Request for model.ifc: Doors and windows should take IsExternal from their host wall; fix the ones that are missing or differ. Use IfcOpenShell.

First a look at what the model holds.

```python
import ifcopenshell
import ifcopenshell.util.element

model = ifcopenshell.open("model.ifc")
print(model.schema)
seen = {}
for e in model.by_type("IfcDoor") + model.by_type("IfcWindow"):
    if not e.FillsVoids:
        continue
    host = e.FillsVoids[0].RelatingOpeningElement.VoidsElements[0].RelatingBuildingElement
    own = ifcopenshell.util.element.get_pset(e, f"Pset_{e.is_a()[3:].removesuffix('StandardCase')}Common", "IsExternal")
    wall = ifcopenshell.util.element.get_pset(host, "Pset_WallCommon", "IsExternal")
    seen[e.is_a(), own, wall] = seen.get((e.is_a(), own, wall), 0) + 1
for (cls, own, wall), count in sorted(seen.items(), key=str):
    print(count, cls, "IsExternal:", own, "| host wall:", wall)
```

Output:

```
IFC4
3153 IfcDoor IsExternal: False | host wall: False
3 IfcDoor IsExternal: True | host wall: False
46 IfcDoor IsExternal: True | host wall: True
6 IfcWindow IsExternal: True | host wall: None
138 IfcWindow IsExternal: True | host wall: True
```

```python
import ifcopenshell
import ifcopenshell.api.pset
import ifcopenshell.util.element

model = ifcopenshell.open("model.ifc")

count = 0
for ifc_class, pset_name in (("IfcDoor", "Pset_DoorCommon"), ("IfcWindow", "Pset_WindowCommon")):
    for e in model.by_type(ifc_class):
        if not e.FillsVoids:
            continue
        host = e.FillsVoids[0].RelatingOpeningElement.VoidsElements[0].RelatingBuildingElement
        external = ifcopenshell.util.element.get_pset(host, "Pset_WallCommon", "IsExternal")
        if external is None or ifcopenshell.util.element.get_pset(e, pset_name, "IsExternal") == external:
            continue
        pset = ifcopenshell.api.pset.add_pset(model, product=e, name=pset_name)
        ifcopenshell.api.pset.edit_pset(model, pset=pset, properties={"IsExternal": external})
        count += 1

print(count, "updated")

model.write("model_v2.ifc")
```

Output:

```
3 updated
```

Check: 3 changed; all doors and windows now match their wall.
